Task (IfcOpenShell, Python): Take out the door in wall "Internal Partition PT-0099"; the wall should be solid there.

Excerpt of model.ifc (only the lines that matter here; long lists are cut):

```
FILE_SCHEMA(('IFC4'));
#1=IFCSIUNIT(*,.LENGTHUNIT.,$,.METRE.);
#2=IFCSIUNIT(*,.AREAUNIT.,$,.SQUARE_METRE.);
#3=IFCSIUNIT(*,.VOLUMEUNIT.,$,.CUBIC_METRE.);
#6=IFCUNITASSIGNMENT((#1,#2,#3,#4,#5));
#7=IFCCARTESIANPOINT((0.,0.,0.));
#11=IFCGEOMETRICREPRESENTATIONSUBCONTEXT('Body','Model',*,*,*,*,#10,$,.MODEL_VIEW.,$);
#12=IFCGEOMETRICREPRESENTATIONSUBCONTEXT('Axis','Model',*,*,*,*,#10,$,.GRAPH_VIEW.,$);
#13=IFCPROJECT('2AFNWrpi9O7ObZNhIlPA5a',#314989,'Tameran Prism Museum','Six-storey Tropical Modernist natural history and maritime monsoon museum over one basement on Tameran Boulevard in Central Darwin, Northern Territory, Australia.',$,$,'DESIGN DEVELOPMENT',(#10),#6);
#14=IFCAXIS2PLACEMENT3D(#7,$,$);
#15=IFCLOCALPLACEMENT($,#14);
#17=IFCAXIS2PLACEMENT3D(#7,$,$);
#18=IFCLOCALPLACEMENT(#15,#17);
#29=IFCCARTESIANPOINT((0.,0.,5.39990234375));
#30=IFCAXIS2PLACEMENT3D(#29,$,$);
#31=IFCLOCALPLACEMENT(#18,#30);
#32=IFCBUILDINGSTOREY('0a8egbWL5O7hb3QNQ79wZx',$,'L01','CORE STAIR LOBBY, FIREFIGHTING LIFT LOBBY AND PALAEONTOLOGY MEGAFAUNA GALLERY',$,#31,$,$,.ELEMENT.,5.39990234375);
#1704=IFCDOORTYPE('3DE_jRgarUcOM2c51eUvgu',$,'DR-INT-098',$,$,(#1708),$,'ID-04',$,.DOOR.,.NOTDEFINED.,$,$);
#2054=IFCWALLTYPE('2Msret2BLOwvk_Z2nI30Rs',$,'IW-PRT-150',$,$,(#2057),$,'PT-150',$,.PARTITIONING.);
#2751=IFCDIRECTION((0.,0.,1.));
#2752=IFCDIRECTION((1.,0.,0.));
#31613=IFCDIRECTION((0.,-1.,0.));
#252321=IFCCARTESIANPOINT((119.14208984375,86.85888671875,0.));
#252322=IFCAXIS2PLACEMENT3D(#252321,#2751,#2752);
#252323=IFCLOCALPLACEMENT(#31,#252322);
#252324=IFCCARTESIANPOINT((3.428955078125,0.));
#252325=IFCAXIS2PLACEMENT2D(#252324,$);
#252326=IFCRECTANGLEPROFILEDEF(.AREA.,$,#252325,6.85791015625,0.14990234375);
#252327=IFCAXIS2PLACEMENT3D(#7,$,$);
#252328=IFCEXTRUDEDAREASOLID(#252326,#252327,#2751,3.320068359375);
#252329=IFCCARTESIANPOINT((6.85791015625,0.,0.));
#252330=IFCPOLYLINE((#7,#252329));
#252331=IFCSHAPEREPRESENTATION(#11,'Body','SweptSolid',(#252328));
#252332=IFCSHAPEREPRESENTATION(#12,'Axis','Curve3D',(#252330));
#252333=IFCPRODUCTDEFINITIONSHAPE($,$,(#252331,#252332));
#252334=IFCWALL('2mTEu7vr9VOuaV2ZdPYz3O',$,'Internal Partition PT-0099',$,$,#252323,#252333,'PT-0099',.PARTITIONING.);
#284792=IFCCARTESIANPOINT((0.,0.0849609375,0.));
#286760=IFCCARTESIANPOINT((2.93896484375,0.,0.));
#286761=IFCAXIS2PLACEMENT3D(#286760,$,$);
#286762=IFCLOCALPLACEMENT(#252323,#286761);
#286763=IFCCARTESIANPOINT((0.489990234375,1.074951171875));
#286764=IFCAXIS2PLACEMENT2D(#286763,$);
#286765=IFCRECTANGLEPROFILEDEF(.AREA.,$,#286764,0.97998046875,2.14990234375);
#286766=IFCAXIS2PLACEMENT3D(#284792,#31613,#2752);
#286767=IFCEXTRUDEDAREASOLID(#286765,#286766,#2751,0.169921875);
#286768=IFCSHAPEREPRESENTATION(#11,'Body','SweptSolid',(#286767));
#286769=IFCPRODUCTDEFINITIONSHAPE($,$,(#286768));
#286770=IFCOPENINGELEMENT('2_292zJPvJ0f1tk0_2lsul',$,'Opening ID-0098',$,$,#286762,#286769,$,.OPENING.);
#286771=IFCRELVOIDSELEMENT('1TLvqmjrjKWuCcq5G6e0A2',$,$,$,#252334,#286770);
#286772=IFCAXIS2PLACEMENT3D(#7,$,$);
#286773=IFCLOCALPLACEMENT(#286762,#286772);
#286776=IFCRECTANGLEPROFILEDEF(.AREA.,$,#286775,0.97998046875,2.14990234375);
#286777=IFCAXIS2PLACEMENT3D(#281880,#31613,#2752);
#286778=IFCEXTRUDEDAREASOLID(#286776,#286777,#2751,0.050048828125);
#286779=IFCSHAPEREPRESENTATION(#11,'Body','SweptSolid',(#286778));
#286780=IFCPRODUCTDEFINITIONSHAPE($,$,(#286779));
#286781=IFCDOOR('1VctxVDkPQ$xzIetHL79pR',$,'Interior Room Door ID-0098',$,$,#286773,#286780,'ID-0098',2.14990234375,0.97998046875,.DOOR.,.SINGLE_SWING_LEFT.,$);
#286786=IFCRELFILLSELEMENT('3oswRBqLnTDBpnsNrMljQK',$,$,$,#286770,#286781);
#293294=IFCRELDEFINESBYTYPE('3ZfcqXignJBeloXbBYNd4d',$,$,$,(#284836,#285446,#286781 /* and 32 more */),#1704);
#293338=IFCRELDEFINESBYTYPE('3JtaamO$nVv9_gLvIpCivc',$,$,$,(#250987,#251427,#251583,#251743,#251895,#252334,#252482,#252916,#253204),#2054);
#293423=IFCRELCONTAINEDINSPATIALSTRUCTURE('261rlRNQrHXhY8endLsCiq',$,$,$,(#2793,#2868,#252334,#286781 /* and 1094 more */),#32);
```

```python
import ifcopenshell
import ifcopenshell.api.feature
import ifcopenshell.api.root
import ifcopenshell.geom
import ifcopenshell.util.shape

model = ifcopenshell.open("model.ifc")
settings = ifcopenshell.geom.settings()


def volume(element):
    """Net volume in cubic metres, openings subtracted."""
    shape = ifcopenshell.geom.create_shape(settings, element)
    return ifcopenshell.util.shape.get_volume(shape.geometry)


door = model.by_guid("1VctxVDkPQ$xzIetHL79pR")
opening = door.FillsVoids[0].RelatingOpeningElement
wall = opening.VoidsElements[0].RelatingBuildingElement
before = volume(wall)

ifcopenshell.api.root.remove_product(model, product=door)
ifcopenshell.api.feature.remove_feature(model, feature=opening)

after = volume(wall)

print(f"wall volume {before:.3f} -> {after:.3f} m3")

model.write("model_rev.ifc")
```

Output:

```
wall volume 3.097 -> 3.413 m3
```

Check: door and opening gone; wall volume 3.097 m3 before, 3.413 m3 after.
